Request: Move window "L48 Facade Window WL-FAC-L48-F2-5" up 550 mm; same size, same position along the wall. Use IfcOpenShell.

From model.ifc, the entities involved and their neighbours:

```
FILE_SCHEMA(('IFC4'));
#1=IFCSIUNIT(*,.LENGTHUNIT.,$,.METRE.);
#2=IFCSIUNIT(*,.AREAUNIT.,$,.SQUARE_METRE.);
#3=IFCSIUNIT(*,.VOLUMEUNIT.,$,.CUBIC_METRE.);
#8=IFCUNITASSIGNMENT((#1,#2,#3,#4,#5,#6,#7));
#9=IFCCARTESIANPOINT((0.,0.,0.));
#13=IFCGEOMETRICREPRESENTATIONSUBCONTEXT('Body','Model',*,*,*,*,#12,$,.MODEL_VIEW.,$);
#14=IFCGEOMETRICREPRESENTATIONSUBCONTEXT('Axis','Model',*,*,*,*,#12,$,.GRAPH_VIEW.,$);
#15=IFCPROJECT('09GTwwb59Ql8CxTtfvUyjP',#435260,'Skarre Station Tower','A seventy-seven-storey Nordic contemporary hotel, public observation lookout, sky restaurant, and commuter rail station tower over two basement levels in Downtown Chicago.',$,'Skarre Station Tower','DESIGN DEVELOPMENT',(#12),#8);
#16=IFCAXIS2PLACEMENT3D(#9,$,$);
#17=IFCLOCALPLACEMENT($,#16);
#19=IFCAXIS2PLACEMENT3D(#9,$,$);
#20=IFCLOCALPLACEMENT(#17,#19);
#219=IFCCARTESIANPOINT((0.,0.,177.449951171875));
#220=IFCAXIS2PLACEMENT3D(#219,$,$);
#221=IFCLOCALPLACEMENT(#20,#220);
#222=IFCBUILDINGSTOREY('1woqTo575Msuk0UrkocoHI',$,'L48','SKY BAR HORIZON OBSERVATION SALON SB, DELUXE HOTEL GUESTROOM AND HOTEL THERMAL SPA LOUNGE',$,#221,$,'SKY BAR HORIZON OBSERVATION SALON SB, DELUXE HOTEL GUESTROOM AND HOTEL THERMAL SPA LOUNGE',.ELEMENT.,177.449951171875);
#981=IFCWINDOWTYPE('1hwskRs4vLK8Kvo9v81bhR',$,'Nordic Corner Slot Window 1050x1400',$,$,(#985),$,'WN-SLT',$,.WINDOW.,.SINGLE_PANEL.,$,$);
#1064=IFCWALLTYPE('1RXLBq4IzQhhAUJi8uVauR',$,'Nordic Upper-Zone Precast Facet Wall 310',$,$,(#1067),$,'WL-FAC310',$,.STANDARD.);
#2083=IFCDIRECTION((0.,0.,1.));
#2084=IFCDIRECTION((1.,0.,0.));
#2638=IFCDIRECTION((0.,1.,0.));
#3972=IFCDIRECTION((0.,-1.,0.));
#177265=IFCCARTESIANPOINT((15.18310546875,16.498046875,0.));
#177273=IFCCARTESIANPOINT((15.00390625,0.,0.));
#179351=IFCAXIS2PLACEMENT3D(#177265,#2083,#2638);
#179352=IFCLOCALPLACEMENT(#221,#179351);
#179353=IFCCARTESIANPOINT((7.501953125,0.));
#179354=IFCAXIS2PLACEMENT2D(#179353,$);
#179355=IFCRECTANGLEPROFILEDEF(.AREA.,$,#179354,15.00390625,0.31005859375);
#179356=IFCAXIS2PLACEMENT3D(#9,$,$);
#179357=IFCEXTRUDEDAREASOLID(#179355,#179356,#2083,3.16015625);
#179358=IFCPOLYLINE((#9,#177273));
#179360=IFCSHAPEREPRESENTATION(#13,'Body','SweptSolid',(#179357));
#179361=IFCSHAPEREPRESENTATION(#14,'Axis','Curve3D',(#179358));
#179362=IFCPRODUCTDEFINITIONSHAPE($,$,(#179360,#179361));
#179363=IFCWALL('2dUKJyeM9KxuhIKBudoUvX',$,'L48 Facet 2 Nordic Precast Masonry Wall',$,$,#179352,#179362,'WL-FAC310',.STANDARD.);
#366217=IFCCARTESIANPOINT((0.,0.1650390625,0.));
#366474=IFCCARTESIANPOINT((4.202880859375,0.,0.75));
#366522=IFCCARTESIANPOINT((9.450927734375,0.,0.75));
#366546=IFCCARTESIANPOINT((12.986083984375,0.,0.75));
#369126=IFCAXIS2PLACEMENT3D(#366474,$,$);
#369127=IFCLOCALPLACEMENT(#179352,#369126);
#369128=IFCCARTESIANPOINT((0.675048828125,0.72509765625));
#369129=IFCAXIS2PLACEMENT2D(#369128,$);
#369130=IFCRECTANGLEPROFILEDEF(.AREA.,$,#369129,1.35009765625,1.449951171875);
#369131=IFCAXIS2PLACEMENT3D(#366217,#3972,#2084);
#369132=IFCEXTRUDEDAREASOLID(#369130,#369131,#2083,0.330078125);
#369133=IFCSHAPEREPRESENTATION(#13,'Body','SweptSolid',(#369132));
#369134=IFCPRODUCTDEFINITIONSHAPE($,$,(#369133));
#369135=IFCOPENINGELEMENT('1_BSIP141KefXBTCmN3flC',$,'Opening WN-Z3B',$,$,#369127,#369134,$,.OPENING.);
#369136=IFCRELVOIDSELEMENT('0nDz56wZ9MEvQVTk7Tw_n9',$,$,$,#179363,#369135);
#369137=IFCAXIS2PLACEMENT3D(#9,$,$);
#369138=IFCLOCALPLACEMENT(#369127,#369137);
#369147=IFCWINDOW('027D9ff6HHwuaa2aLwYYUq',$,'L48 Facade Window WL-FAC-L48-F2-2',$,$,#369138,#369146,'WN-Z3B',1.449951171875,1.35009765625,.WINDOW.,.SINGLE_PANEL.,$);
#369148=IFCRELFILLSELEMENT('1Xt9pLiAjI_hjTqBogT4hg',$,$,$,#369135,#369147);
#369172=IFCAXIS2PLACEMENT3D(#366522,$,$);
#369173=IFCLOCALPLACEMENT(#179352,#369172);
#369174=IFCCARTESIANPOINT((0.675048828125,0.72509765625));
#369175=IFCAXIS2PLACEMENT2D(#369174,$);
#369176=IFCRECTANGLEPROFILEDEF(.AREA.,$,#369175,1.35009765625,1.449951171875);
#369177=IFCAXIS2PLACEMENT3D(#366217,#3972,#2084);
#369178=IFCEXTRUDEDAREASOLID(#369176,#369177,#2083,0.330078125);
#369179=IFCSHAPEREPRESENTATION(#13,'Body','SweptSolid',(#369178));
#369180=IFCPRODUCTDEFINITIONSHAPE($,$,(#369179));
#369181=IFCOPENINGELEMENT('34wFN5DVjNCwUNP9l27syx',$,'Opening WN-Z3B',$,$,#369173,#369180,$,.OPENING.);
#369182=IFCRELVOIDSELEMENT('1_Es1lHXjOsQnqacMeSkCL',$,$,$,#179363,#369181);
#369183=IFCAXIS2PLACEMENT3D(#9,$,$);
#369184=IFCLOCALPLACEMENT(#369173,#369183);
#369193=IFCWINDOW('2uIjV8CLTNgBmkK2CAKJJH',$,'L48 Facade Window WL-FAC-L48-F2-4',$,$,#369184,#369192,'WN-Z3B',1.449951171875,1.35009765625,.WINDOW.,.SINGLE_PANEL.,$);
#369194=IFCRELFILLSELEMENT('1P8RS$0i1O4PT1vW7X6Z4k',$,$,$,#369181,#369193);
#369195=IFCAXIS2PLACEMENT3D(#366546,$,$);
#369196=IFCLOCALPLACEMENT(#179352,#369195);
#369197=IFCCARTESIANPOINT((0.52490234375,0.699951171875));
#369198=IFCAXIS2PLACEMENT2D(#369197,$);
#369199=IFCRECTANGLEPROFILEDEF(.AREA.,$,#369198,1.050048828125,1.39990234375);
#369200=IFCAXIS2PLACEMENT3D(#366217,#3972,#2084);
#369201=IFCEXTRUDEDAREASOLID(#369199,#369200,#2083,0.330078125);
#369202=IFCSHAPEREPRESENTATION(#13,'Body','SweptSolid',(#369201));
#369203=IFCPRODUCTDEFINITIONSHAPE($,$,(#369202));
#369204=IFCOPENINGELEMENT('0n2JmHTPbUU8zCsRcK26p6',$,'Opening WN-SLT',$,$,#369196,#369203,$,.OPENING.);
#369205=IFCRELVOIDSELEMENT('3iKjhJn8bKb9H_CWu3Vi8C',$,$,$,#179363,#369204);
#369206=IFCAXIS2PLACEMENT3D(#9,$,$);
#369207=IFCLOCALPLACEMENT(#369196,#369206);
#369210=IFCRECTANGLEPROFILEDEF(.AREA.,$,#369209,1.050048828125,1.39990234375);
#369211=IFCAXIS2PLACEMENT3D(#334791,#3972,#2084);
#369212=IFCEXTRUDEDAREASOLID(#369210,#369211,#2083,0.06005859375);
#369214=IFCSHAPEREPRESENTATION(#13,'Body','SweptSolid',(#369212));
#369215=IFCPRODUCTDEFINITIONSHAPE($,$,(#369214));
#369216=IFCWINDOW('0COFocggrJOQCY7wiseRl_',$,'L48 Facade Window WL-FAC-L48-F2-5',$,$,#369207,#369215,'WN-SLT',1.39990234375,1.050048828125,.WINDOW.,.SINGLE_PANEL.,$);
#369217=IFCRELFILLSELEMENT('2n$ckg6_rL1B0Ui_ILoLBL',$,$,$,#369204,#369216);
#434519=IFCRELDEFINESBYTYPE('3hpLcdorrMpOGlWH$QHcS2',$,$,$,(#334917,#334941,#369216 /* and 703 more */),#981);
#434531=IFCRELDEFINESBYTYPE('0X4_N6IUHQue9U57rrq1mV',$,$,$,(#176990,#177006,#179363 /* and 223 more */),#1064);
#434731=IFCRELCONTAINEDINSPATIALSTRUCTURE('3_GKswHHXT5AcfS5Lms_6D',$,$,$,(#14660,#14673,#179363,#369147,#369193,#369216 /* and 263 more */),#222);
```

```python
import numpy as np
import ifcopenshell
import ifcopenshell.api.geometry
import ifcopenshell.util.placement
import ifcopenshell.util.unit

model = ifcopenshell.open("model.ifc")
unit_scale = ifcopenshell.util.unit.calculate_unit_scale(model)

window = model.by_guid("0COFocggrJOQCY7wiseRl_")
opening = window.FillsVoids[0].RelatingOpeningElement
dz = 0.55

shift = np.array([0.0, 0.0, dz])
# The window is placed relative to its opening, so it follows when the opening moves.
matrix = ifcopenshell.util.placement.get_local_placement(opening.ObjectPlacement)
matrix[:3, 3] += shift
ifcopenshell.api.geometry.edit_object_placement(
    model, product=opening, matrix=matrix, is_si=False, should_transform_children=True
)

print(f"moved by {dz * unit_scale:+.3f} m")

model.write("model_v2.ifc")
```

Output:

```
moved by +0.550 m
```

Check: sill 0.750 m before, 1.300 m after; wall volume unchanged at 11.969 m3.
